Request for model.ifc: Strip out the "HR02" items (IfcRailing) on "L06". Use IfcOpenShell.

First a look at what the model holds.

```python
import ifcopenshell
import ifcopenshell.util.element

model = ifcopenshell.open("model.ifc")
print(model.schema)
storey = next(s for s in model.by_type("IfcBuildingStorey") if s.Name == "L06")
railings = [e for e in ifcopenshell.util.element.get_decomposition(storey) if e.is_a("IfcRailing")]
seen = {}
for e in railings:
    element_type = ifcopenshell.util.element.get_type(e)
    name = element_type.Name if element_type not in (None, e) else None
    seen[name] = seen.get(name, 0) + 1
for name, count in sorted(seen.items(), key=str):
    print(count, "x", name)
```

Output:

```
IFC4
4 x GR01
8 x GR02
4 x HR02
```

```python
import ifcopenshell
import ifcopenshell.api.root
import ifcopenshell.util.element

model = ifcopenshell.open("model.ifc")

storey = next(s for s in model.by_type("IfcBuildingStorey") if s.Name == "L06")
railings = [e for e in ifcopenshell.util.element.get_decomposition(storey) if e.is_a("IfcRailing")]
targets = [e for e in railings if (t := ifcopenshell.util.element.get_type(e)) not in (None, e) and t.Name == "HR02"]

for e in targets:
    ifcopenshell.api.root.remove_product(model, product=e)
print(len(targets), "removed")

model.write("model_updated.ifc")
```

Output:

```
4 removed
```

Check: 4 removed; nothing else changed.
